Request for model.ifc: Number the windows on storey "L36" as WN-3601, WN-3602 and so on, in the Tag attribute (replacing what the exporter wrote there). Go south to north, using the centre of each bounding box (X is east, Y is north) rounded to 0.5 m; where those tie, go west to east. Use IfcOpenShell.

First a look at what the model holds.

```python
import ifcopenshell
import ifcopenshell.util.element
import ifcopenshell.util.placement

model = ifcopenshell.open("model.ifc")
print(model.schema)
storey = next(s for s in model.by_type("IfcBuildingStorey") if s.Name == "L36")
windows = [e for e in ifcopenshell.util.element.get_decomposition(storey) if e.is_a("IfcWindow")]
for e in sorted(windows, key=lambda e: e.id()):
    origin = ifcopenshell.util.placement.get_local_placement(e.ObjectPlacement)[:3, 3]
    print(e.id(), e.Tag, e.Name, origin.round(2) + 0.0, sep=" | ")
```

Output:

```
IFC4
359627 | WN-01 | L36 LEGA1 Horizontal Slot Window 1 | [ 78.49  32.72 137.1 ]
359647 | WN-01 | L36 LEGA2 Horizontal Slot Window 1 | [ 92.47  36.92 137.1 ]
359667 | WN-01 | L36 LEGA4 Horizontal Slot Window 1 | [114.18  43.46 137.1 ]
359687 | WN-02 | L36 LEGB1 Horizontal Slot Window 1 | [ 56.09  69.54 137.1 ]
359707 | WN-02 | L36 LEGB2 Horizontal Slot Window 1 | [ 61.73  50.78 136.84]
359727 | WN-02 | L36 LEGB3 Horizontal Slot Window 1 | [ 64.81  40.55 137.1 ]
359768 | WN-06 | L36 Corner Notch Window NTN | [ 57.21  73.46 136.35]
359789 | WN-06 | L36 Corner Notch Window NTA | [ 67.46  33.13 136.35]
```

```python
import ifcopenshell
import ifcopenshell.geom
import ifcopenshell.util.element
import ifcopenshell.util.shape

model = ifcopenshell.open("model.ifc")
settings = ifcopenshell.geom.settings()
settings.set("use-world-coords", True)


def centre(element):
    shape = ifcopenshell.geom.create_shape(settings, element)
    return ifcopenshell.util.shape.get_bbox_centroid(shape.geometry)


storey = next(s for s in model.by_type("IfcBuildingStorey") if s.Name == "L36")
windows = [e for e in ifcopenshell.util.element.get_decomposition(storey) if e.is_a("IfcWindow")]

# Insertion points can sit at a corner or the storey origin, so sort by the geometry (in metres).
centres = {e: centre(e) for e in windows}
windows.sort(key=lambda e: (round(centres[e][1] / 0.5), centres[e][0]))

for i, e in enumerate(windows, start=1):
    number = f"WN-36{i:02d}"
    e.Tag = number
    print(e.id(), number)

model.write("model_edited.ifc")
```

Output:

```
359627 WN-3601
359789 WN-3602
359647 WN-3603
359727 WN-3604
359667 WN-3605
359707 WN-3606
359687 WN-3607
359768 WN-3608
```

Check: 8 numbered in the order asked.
